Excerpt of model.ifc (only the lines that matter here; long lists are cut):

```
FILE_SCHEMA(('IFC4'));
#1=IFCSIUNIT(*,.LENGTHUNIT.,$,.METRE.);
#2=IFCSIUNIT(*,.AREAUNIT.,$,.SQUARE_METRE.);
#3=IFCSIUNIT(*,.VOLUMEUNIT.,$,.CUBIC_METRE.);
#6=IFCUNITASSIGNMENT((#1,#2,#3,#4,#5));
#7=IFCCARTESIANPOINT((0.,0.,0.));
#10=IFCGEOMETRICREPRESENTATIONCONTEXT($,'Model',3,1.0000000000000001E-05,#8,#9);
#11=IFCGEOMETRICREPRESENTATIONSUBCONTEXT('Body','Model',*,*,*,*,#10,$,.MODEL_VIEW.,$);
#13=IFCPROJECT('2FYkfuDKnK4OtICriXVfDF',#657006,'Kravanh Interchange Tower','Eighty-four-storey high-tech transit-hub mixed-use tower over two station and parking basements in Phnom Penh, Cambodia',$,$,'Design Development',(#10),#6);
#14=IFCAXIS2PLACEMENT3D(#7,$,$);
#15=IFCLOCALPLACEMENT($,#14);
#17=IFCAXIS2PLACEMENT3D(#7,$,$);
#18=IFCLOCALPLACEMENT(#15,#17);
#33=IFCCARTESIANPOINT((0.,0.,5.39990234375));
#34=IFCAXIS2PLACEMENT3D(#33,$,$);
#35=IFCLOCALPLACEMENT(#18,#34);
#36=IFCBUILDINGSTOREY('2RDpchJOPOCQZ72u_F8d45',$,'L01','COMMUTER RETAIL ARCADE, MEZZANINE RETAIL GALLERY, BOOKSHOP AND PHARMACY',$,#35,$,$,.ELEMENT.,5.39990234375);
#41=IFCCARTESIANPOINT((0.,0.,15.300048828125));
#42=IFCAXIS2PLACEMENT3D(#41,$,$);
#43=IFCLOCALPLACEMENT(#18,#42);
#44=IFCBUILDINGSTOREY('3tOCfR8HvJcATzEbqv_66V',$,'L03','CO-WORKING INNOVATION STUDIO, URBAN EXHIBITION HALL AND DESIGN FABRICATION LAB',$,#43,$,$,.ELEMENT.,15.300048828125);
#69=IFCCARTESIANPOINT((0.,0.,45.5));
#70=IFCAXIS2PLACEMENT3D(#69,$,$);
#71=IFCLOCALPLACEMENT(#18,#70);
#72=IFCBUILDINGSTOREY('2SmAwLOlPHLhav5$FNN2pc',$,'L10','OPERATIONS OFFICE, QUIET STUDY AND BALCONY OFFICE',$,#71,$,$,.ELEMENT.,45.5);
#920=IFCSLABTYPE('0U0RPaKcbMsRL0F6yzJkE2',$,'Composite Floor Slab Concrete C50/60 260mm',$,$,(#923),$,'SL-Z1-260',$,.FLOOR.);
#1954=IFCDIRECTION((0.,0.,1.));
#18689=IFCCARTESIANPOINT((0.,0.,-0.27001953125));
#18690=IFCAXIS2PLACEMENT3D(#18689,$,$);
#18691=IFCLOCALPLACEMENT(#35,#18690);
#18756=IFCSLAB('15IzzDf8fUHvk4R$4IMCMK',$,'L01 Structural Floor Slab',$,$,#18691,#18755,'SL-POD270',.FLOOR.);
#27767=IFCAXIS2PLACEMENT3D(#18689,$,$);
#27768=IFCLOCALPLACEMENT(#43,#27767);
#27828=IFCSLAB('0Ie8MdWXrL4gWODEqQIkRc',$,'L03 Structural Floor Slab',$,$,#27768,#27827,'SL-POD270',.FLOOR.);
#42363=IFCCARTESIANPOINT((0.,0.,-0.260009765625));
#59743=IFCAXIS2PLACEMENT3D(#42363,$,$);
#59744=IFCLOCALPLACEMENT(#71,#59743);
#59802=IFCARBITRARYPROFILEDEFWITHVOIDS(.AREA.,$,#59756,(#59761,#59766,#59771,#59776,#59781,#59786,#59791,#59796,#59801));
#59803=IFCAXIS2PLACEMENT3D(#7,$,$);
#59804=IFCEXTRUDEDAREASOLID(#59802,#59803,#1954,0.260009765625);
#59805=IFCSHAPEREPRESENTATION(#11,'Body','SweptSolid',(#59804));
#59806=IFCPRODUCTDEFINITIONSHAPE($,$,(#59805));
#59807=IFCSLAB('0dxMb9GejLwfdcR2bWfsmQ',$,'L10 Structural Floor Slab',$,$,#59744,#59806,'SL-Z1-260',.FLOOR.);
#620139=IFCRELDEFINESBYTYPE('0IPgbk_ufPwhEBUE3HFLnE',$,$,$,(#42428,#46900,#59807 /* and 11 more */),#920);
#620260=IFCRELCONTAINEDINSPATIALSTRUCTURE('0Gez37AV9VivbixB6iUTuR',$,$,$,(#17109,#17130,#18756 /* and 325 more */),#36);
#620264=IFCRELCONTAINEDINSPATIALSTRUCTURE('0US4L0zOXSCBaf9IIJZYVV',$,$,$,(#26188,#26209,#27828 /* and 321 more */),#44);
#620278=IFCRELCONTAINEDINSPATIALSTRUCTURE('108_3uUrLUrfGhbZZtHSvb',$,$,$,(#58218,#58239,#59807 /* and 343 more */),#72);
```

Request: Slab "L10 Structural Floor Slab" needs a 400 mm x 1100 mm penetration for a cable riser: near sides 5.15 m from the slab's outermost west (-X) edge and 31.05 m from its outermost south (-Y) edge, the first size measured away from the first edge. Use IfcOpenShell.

```python
import numpy as np
import ifcopenshell
import ifcopenshell.api.feature
import ifcopenshell.api.geometry
import ifcopenshell.api.root
import ifcopenshell.geom
import ifcopenshell.util.placement
import ifcopenshell.util.representation
import ifcopenshell.util.shape
import ifcopenshell.util.unit

model = ifcopenshell.open("model.ifc")
unit_scale = ifcopenshell.util.unit.calculate_unit_scale(model)
settings = ifcopenshell.geom.settings()


def volume(element):
    """Net volume in cubic metres, openings subtracted."""
    shape = ifcopenshell.geom.create_shape(settings, element)
    return ifcopenshell.util.shape.get_volume(shape.geometry)


slab = model.by_guid("0dxMb9GejLwfdcR2bWfsmQ")
before = volume(slab)

# Extent in the slab's own axes, in metres. The edges named are its -X and -Y sides.
slab_shape = ifcopenshell.geom.create_shape(settings, slab)
vertices = ifcopenshell.util.shape.get_vertices(slab_shape.geometry)
x_min, y_min, bottom = vertices.min(axis=0)
top = vertices[:, 2].max()

opening = ifcopenshell.api.root.create_entity(model, ifc_class="IfcOpeningElement", name="Cable riser opening", predefined_type="OPENING")
context = ifcopenshell.util.representation.get_context(model, "Model", "Body", "MODEL_VIEW")
width, depth = 0.4, 1.1
outline = [(0.0, 0.0), (width, 0.0), (width, depth), (0.0, depth), (0.0, 0.0)]
# Overshoot both faces by 50 mm so the cut is clean.
shape = ifcopenshell.api.geometry.add_slab_representation(
    model, context=context, depth=top - bottom + 0.1, polyline=outline
)
ifcopenshell.api.geometry.assign_representation(model, product=opening, representation=shape)

matrix = ifcopenshell.util.placement.get_local_placement(slab.ObjectPlacement)
matrix[:, 3] = matrix @ np.append(np.array([x_min + 5.15, y_min + 31.05, bottom - 0.05]) / unit_scale, 1.0)
ifcopenshell.api.geometry.edit_object_placement(model, product=opening, matrix=matrix, is_si=False)
ifcopenshell.api.feature.add_feature(model, feature=opening, element=slab)

after = volume(slab)

print(f"slab volume {before:.3f} -> {after:.3f} m3")

model.write("model_v2.ifc")
```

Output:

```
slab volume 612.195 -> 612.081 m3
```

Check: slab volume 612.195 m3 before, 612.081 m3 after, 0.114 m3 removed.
